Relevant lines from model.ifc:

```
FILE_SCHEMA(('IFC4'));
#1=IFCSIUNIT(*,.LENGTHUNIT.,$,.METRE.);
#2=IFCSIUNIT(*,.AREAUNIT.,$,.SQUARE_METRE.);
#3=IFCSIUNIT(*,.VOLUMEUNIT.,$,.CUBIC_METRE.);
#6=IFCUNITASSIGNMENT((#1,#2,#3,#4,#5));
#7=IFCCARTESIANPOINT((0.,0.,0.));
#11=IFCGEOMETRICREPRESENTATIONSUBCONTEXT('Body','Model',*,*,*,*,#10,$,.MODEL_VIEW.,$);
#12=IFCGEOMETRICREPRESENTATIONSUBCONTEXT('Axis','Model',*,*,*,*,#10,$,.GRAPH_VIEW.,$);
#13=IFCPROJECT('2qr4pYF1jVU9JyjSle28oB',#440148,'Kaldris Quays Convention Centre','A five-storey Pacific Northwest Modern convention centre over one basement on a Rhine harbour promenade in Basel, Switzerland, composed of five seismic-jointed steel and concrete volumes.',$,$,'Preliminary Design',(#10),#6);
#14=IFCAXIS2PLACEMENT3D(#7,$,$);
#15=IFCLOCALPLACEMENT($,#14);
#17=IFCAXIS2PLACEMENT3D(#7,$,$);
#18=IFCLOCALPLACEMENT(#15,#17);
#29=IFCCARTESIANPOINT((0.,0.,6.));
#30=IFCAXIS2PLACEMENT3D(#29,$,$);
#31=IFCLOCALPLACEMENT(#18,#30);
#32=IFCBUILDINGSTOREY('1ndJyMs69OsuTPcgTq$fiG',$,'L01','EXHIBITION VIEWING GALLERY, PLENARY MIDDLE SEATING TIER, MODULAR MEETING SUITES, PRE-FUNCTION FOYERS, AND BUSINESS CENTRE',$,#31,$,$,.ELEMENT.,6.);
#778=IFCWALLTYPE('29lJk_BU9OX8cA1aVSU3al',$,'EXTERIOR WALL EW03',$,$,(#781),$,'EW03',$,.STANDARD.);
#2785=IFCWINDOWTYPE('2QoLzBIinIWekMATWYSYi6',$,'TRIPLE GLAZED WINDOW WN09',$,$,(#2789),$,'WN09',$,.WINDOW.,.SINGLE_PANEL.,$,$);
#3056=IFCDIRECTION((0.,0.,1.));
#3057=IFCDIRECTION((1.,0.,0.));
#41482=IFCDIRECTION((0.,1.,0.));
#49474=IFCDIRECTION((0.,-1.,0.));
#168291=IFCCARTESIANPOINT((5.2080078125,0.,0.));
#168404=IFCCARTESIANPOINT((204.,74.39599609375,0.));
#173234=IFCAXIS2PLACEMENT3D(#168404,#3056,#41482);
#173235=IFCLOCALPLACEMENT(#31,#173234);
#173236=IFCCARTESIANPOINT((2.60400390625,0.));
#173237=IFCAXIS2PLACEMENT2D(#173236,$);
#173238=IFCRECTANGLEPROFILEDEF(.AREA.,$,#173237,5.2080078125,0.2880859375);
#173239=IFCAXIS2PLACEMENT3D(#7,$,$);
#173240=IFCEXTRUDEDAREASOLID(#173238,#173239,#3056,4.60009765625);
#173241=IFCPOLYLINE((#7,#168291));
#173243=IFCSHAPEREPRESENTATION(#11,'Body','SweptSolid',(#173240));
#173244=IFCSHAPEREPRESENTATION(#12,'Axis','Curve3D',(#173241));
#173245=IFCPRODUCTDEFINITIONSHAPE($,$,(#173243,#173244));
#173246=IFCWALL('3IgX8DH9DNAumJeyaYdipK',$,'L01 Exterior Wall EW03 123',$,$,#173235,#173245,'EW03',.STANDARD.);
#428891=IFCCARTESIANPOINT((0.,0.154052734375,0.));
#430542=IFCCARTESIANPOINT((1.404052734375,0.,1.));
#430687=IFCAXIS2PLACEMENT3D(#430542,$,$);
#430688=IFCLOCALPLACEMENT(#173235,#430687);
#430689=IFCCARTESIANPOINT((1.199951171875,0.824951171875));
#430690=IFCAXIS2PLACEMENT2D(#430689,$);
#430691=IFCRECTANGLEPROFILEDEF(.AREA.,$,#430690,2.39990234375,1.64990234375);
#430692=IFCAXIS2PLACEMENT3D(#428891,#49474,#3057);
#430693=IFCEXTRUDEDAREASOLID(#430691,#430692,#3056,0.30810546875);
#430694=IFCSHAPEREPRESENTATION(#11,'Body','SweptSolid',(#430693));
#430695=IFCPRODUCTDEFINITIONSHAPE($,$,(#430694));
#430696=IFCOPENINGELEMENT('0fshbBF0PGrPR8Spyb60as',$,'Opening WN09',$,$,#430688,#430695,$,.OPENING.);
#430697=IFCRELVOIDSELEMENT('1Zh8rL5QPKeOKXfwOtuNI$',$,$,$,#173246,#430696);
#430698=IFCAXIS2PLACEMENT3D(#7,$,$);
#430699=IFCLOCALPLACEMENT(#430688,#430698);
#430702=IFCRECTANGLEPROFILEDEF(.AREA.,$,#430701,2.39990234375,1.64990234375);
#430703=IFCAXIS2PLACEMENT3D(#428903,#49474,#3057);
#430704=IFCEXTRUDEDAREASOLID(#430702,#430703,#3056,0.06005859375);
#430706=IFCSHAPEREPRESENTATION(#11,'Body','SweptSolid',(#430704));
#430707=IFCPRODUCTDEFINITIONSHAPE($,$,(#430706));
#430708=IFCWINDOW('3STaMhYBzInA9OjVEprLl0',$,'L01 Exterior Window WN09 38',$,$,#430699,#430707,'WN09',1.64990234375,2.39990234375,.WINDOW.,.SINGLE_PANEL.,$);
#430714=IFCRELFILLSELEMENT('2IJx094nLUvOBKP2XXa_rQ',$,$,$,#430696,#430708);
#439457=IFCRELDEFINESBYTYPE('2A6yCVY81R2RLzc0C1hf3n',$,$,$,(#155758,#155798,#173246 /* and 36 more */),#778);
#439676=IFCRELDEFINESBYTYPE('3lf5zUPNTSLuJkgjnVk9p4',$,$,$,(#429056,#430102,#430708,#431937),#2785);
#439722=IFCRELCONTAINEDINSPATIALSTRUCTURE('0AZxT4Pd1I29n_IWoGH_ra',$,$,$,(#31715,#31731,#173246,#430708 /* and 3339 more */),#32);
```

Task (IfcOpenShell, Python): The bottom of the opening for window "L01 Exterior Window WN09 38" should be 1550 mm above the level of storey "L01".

```python
import numpy as np
import ifcopenshell
import ifcopenshell.api.geometry
import ifcopenshell.geom
import ifcopenshell.util.element
import ifcopenshell.util.placement
import ifcopenshell.util.shape
import ifcopenshell.util.unit

model = ifcopenshell.open("model.ifc")
unit_scale = ifcopenshell.util.unit.calculate_unit_scale(model)

window = model.by_id(430708)
opening = window.FillsVoids[0].RelatingOpeningElement
storey = ifcopenshell.util.element.get_container(window, ifc_class="IfcBuildingStorey")
level = ifcopenshell.util.placement.get_local_placement(storey.ObjectPlacement)[2, 3]

# The opening's origin need not be at the sill, so measure its lowest point.
shape = ifcopenshell.geom.create_shape(ifcopenshell.geom.settings(), opening)
bottom = ifcopenshell.util.shape.get_shape_bottom_elevation(shape, shape.geometry) / unit_scale
dz = level + 1.55 / unit_scale - bottom

shift = np.array([0.0, 0.0, dz])
# The window is placed relative to its opening, so it follows when the opening moves.
matrix = ifcopenshell.util.placement.get_local_placement(opening.ObjectPlacement)
matrix[:3, 3] += shift
ifcopenshell.api.geometry.edit_object_placement(
    model, product=opening, matrix=matrix, is_si=False, should_transform_children=True
)

print(f"moved by {dz * unit_scale:+.3f} m")

model.write("model_updated.ifc")
```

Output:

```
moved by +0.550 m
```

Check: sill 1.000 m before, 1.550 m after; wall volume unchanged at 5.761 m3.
